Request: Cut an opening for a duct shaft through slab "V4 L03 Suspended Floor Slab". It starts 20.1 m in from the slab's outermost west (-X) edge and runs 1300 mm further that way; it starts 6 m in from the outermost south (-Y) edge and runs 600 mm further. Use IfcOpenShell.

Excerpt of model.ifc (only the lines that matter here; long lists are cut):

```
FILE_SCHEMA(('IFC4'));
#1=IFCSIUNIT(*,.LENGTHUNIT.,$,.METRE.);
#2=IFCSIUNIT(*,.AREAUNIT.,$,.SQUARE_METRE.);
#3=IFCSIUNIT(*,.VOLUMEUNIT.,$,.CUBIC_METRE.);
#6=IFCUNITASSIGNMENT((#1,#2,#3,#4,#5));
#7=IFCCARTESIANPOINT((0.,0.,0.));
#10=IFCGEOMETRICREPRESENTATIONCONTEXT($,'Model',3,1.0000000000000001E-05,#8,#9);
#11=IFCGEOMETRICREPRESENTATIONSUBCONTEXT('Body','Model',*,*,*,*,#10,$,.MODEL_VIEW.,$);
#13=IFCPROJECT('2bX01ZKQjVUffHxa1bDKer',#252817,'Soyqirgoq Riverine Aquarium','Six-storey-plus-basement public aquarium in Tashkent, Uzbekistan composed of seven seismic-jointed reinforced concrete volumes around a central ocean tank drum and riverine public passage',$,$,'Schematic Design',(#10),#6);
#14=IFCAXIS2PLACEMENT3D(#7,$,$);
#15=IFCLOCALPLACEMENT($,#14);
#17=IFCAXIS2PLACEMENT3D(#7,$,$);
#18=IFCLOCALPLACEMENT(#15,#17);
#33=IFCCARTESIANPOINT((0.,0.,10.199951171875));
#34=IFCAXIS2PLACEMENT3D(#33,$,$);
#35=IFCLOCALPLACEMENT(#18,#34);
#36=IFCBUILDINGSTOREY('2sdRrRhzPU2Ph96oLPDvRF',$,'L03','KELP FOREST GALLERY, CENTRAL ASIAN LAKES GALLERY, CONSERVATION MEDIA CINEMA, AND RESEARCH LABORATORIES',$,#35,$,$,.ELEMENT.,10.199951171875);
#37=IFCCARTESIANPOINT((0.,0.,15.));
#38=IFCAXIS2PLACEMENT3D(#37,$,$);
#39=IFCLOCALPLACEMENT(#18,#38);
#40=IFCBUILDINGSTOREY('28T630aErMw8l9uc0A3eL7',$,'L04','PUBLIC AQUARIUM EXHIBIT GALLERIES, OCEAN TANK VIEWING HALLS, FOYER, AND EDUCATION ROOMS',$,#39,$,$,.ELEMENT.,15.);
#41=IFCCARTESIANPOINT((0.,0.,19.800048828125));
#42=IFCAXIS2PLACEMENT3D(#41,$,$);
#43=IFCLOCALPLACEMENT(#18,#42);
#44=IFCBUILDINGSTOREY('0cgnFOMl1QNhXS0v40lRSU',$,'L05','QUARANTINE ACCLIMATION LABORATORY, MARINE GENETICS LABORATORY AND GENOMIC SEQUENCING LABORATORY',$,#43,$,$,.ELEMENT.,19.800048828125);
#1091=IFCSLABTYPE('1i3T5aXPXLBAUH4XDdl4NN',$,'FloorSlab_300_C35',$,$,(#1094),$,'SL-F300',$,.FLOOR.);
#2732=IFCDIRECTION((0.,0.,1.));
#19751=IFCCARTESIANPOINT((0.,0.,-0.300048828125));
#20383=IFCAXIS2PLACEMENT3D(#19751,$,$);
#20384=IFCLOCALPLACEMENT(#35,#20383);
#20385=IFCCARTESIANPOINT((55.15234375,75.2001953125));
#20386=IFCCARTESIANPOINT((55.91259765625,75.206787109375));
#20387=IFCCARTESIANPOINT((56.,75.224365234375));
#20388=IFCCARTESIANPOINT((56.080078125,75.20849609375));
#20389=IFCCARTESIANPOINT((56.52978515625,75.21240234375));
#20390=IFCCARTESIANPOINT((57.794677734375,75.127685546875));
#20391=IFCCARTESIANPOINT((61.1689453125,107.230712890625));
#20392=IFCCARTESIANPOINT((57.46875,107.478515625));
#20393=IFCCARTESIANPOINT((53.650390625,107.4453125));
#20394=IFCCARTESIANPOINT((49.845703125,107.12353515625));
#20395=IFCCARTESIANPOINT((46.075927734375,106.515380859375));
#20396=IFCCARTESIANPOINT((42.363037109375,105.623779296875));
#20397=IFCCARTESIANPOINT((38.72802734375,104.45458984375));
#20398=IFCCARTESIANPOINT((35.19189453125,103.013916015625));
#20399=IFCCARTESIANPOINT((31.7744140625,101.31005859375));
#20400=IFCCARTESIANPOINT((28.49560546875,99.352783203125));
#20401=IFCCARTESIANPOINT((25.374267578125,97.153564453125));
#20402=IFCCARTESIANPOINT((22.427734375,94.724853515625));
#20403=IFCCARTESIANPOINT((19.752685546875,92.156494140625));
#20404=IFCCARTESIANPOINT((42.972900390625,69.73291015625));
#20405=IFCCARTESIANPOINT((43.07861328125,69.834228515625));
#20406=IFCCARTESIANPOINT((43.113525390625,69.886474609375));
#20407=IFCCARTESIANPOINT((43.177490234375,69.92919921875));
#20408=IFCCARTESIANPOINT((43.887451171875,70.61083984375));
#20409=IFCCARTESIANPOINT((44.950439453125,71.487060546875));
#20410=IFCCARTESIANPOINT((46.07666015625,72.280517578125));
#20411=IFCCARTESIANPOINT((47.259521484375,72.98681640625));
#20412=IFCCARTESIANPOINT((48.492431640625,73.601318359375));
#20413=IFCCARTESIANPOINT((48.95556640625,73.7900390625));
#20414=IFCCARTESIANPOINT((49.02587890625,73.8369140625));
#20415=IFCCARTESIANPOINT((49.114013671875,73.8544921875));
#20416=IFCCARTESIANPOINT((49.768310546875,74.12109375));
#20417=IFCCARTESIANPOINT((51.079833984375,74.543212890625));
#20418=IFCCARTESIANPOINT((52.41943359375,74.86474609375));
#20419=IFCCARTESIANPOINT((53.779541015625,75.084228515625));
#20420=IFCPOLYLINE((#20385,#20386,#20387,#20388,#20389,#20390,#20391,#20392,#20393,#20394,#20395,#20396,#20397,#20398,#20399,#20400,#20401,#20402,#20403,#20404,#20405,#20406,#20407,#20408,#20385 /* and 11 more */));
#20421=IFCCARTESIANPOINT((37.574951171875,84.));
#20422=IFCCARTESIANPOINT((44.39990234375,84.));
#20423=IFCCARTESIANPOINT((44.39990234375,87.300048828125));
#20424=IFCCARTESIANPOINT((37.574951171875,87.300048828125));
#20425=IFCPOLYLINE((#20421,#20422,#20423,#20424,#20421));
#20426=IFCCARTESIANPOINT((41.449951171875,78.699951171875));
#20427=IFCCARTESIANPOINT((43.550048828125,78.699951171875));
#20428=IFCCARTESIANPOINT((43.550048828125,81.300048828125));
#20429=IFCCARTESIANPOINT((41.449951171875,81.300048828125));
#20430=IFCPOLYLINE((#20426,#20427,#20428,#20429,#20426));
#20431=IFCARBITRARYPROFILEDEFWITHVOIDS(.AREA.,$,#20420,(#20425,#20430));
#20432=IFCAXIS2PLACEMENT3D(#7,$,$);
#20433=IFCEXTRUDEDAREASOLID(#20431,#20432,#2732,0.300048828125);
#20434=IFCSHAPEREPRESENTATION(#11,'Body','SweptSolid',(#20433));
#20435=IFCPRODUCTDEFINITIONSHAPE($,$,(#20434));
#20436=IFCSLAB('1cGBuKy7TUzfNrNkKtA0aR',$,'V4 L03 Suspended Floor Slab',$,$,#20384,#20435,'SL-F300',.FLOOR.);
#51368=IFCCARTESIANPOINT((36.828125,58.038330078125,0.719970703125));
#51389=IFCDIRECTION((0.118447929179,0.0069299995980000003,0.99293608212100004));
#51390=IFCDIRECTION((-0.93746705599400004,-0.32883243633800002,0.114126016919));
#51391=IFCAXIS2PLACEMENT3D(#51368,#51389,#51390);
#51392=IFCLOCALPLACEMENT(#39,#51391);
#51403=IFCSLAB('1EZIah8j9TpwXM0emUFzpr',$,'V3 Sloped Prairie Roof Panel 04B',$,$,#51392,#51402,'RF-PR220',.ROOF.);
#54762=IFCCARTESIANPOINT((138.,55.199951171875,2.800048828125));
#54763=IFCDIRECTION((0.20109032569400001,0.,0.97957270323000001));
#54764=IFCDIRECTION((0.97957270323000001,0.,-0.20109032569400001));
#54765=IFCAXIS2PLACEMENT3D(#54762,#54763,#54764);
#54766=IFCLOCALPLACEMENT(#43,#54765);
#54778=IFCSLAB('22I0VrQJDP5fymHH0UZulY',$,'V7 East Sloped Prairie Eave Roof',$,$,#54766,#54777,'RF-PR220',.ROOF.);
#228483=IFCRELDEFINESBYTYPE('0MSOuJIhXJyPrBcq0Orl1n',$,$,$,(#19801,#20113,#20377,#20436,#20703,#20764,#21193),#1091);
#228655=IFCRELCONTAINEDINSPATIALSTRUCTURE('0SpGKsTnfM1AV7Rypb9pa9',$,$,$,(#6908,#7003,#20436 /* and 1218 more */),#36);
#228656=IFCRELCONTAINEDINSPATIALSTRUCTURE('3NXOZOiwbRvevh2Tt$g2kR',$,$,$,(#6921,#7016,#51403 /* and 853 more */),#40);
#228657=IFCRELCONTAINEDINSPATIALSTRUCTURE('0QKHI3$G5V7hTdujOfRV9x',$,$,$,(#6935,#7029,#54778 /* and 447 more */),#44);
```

```python
import numpy as np
import ifcopenshell
import ifcopenshell.api.feature
import ifcopenshell.api.geometry
import ifcopenshell.api.root
import ifcopenshell.geom
import ifcopenshell.util.placement
import ifcopenshell.util.representation
import ifcopenshell.util.shape
import ifcopenshell.util.unit

model = ifcopenshell.open("model.ifc")
unit_scale = ifcopenshell.util.unit.calculate_unit_scale(model)
settings = ifcopenshell.geom.settings()


def volume(element):
    """Net volume in cubic metres, openings subtracted."""
    shape = ifcopenshell.geom.create_shape(settings, element)
    return ifcopenshell.util.shape.get_volume(shape.geometry)


slab = model.by_guid("1cGBuKy7TUzfNrNkKtA0aR")
before = volume(slab)

# Extent in the slab's own axes, in metres. The edges named are its -X and -Y sides.
slab_shape = ifcopenshell.geom.create_shape(settings, slab)
vertices = ifcopenshell.util.shape.get_vertices(slab_shape.geometry)
x_min, y_min, bottom = vertices.min(axis=0)
top = vertices[:, 2].max()

opening = ifcopenshell.api.root.create_entity(model, ifc_class="IfcOpeningElement", name="Duct shaft opening", predefined_type="OPENING")
context = ifcopenshell.util.representation.get_context(model, "Model", "Body", "MODEL_VIEW")
width, depth = 1.3, 0.6
outline = [(0.0, 0.0), (width, 0.0), (width, depth), (0.0, depth), (0.0, 0.0)]
# Overshoot both faces by 50 mm so the cut is clean.
shape = ifcopenshell.api.geometry.add_slab_representation(
    model, context=context, depth=top - bottom + 0.1, polyline=outline
)
ifcopenshell.api.geometry.assign_representation(model, product=opening, representation=shape)

matrix = ifcopenshell.util.placement.get_local_placement(slab.ObjectPlacement)
matrix[:, 3] = matrix @ np.append(np.array([x_min + 20.1, y_min + 6, bottom - 0.05]) / unit_scale, 1.0)
ifcopenshell.api.geometry.edit_object_placement(model, product=opening, matrix=matrix, is_si=False)
ifcopenshell.api.feature.add_feature(model, feature=opening, element=slab)

after = volume(slab)

print(f"slab volume {before:.3f} -> {after:.3f} m3")

model.write("model_rev.ifc")
```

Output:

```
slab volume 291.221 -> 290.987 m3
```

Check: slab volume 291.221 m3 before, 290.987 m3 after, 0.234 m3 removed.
